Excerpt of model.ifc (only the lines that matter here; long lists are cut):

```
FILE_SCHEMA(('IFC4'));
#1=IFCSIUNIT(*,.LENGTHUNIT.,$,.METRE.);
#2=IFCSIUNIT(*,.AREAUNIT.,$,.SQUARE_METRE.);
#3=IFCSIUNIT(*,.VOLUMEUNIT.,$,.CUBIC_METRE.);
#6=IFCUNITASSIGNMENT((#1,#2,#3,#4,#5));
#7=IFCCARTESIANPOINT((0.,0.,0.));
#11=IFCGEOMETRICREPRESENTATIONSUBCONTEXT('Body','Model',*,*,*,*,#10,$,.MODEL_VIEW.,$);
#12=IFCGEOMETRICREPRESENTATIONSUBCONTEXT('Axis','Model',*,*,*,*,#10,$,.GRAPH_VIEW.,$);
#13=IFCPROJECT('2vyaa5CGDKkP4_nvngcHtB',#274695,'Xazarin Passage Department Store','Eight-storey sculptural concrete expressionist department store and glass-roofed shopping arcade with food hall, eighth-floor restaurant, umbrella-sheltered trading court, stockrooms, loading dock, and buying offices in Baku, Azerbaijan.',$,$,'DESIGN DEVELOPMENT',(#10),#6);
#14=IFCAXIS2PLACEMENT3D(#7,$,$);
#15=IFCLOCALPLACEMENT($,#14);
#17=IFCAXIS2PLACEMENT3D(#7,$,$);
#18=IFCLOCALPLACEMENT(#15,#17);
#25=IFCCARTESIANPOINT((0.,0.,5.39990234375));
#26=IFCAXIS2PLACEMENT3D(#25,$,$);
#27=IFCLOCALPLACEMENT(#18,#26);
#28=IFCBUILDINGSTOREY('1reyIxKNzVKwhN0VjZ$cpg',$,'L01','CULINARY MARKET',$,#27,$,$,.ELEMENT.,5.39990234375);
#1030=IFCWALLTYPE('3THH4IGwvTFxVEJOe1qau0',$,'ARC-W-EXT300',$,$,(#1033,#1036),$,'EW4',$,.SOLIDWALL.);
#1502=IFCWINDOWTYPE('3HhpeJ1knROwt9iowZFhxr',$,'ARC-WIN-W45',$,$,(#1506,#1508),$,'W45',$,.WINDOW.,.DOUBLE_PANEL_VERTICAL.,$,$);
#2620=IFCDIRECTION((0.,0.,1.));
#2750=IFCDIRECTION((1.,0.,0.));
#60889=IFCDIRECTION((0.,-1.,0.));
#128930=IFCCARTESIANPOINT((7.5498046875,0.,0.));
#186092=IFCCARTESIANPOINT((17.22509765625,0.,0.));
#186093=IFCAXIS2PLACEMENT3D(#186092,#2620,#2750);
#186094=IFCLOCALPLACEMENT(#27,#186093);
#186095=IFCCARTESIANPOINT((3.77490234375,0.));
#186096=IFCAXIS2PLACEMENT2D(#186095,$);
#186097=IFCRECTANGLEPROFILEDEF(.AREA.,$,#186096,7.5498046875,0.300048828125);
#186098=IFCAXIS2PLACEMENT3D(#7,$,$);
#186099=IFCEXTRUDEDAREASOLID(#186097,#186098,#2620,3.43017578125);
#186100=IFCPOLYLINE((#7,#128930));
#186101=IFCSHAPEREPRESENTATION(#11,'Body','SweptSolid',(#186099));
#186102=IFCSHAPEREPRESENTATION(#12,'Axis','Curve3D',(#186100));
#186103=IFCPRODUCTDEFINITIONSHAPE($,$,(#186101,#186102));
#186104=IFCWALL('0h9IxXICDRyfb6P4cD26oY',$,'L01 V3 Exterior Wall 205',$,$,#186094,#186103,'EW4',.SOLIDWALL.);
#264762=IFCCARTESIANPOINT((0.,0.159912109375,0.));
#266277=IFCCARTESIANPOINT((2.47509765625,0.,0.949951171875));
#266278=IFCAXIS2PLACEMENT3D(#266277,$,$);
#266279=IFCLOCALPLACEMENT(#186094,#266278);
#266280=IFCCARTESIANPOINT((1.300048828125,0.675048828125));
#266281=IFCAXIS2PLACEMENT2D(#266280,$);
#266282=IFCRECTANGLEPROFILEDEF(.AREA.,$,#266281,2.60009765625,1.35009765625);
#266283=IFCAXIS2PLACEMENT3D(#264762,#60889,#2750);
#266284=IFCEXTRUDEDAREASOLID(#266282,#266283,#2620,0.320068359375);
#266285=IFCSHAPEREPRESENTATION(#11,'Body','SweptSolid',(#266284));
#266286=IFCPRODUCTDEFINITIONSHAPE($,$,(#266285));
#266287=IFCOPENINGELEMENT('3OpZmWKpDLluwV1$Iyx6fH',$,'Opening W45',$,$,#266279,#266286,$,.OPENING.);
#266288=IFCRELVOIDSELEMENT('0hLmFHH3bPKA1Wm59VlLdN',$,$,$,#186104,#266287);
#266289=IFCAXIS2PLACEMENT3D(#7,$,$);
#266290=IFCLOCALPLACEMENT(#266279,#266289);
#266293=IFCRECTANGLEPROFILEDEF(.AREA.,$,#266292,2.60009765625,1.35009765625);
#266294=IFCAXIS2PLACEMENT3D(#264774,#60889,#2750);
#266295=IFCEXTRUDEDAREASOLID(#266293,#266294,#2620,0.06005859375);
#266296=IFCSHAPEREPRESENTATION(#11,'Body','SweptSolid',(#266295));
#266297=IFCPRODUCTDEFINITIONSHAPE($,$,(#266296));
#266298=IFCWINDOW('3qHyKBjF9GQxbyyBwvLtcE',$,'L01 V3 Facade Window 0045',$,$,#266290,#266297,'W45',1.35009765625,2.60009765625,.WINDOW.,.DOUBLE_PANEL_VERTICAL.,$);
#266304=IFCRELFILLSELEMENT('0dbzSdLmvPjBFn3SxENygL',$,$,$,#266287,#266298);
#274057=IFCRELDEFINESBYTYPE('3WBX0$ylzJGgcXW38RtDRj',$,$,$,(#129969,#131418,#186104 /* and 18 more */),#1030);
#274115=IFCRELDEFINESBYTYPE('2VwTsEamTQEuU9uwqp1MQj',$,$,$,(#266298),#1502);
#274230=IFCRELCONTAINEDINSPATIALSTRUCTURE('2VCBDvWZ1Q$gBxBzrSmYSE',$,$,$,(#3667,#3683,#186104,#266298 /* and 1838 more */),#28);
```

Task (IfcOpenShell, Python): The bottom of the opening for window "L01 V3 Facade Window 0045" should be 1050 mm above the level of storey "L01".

```python
import numpy as np
import ifcopenshell
import ifcopenshell.api.geometry
import ifcopenshell.geom
import ifcopenshell.util.element
import ifcopenshell.util.placement
import ifcopenshell.util.shape
import ifcopenshell.util.unit

model = ifcopenshell.open("model.ifc")
unit_scale = ifcopenshell.util.unit.calculate_unit_scale(model)

window = model.by_guid("3qHyKBjF9GQxbyyBwvLtcE")
opening = window.FillsVoids[0].RelatingOpeningElement
storey = ifcopenshell.util.element.get_container(window, ifc_class="IfcBuildingStorey")
level = ifcopenshell.util.placement.get_local_placement(storey.ObjectPlacement)[2, 3]

# The opening's origin need not be at the sill, so measure its lowest point.
shape = ifcopenshell.geom.create_shape(ifcopenshell.geom.settings(), opening)
bottom = ifcopenshell.util.shape.get_shape_bottom_elevation(shape, shape.geometry) / unit_scale
dz = level + 1.05 - bottom

shift = np.array([0.0, 0.0, dz])
# The window is placed relative to its opening, so it follows when the opening moves.
matrix = ifcopenshell.util.placement.get_local_placement(opening.ObjectPlacement)
matrix[:3, 3] += shift
ifcopenshell.api.geometry.edit_object_placement(
    model, product=opening, matrix=matrix, is_si=False, should_transform_children=True
)

print(f"moved by {dz * unit_scale:+.3f} m")

model.write("model_rev.ifc")
```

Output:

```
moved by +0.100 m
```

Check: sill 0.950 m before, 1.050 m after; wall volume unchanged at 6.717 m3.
